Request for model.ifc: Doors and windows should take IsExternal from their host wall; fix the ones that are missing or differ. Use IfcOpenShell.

First a look at what the model holds.

```python
import ifcopenshell
import ifcopenshell.util.element

model = ifcopenshell.open("model.ifc")
print(model.schema)
seen = {}
for e in model.by_type("IfcDoor") + model.by_type("IfcWindow"):
    if not e.FillsVoids:
        continue
    host = e.FillsVoids[0].RelatingOpeningElement.VoidsElements[0].RelatingBuildingElement
    own = ifcopenshell.util.element.get_pset(e, f"Pset_{e.is_a()[3:].removesuffix('StandardCase')}Common", "IsExternal")
    wall = ifcopenshell.util.element.get_pset(host, "Pset_WallCommon", "IsExternal")
    seen[e.is_a(), own, wall] = seen.get((e.is_a(), own, wall), 0) + 1
for (cls, own, wall), count in sorted(seen.items(), key=str):
    print(count, cls, "IsExternal:", own, "| host wall:", wall)
```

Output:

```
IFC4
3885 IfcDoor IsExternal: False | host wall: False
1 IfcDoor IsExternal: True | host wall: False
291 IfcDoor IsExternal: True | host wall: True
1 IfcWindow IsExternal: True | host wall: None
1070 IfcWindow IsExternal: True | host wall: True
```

```python
import ifcopenshell
import ifcopenshell.api.pset
import ifcopenshell.util.element

model = ifcopenshell.open("model.ifc")

count = 0
for ifc_class, pset_name in (("IfcDoor", "Pset_DoorCommon"), ("IfcWindow", "Pset_WindowCommon")):
    for e in model.by_type(ifc_class):
        if not e.FillsVoids:
            continue
        host = e.FillsVoids[0].RelatingOpeningElement.VoidsElements[0].RelatingBuildingElement
        external = ifcopenshell.util.element.get_pset(host, "Pset_WallCommon", "IsExternal")
        if external is None or ifcopenshell.util.element.get_pset(e, pset_name, "IsExternal") == external:
            continue
        pset = ifcopenshell.api.pset.add_pset(model, product=e, name=pset_name)
        ifcopenshell.api.pset.edit_pset(model, pset=pset, properties={"IsExternal": external})
        count += 1

print(count, "updated")

model.write("model_rev.ifc")
```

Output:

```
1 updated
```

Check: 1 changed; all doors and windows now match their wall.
